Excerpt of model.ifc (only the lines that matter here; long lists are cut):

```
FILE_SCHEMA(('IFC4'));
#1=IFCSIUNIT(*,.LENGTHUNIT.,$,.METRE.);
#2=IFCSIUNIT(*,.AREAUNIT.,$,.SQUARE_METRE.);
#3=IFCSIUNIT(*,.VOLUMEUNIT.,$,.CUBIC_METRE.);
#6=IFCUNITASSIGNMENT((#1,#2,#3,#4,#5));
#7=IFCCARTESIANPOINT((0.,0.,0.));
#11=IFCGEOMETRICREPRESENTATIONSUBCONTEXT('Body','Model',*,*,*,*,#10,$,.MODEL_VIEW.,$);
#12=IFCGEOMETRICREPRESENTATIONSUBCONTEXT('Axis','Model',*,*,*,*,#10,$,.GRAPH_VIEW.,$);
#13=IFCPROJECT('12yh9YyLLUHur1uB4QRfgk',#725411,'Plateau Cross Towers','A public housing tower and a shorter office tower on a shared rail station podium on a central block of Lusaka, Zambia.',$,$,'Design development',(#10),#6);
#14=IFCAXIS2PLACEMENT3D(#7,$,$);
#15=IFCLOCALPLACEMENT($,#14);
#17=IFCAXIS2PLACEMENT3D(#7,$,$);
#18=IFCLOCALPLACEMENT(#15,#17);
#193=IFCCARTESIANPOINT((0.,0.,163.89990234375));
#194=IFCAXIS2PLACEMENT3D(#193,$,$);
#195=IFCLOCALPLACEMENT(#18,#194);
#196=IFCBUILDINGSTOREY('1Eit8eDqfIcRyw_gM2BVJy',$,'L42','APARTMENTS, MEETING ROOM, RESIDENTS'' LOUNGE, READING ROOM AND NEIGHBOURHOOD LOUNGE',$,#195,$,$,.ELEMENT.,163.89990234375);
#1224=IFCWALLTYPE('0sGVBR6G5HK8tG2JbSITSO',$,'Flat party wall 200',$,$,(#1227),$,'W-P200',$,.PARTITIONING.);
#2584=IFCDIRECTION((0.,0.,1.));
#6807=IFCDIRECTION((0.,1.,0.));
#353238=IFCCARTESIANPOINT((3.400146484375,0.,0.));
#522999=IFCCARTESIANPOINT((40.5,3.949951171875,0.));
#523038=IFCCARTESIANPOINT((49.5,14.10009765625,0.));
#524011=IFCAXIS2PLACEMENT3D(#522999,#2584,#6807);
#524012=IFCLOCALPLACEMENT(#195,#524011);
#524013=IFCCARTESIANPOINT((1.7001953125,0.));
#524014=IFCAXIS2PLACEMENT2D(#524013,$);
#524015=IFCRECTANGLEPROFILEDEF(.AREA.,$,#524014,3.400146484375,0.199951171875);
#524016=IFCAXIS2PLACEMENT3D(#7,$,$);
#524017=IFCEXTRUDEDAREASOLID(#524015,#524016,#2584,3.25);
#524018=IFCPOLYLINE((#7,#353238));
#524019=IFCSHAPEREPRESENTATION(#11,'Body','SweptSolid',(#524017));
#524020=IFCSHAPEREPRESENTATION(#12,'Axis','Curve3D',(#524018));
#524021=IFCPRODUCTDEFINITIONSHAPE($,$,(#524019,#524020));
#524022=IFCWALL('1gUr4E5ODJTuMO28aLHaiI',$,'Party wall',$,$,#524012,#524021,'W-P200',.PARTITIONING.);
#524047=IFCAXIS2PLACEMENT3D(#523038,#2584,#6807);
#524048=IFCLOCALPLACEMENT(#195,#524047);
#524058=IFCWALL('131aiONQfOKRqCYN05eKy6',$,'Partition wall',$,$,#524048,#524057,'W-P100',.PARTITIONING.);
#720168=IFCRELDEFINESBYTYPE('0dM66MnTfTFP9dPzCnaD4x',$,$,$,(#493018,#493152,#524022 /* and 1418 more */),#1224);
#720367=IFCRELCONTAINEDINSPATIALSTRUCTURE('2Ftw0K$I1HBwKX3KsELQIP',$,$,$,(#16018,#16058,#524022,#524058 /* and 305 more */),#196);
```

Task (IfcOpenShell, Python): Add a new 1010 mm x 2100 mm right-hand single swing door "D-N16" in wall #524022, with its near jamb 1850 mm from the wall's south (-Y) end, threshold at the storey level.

```python
import numpy as np
import ifcopenshell
import ifcopenshell.api.feature
import ifcopenshell.api.geometry
import ifcopenshell.api.root
import ifcopenshell.api.spatial
import ifcopenshell.geom
import ifcopenshell.util.element
import ifcopenshell.util.placement
import ifcopenshell.util.representation
import ifcopenshell.util.shape
import ifcopenshell.util.unit

model = ifcopenshell.open("model.ifc")
unit_scale = ifcopenshell.util.unit.calculate_unit_scale(model)
settings = ifcopenshell.geom.settings()


def volume(element):
    """Net volume in cubic metres, openings subtracted."""
    shape = ifcopenshell.geom.create_shape(settings, element)
    return ifcopenshell.util.shape.get_volume(shape.geometry)


wall = model.by_id(524022)
storey = ifcopenshell.util.element.get_container(wall, ifc_class="IfcBuildingStorey")
context = ifcopenshell.util.representation.get_context(model, "Model", "Body", "MODEL_VIEW")
before = volume(wall)

width, height, from_end, sill = 1.01, 2.1, 1.85, 0.0  # metres

# The wall runs along its own X axis, and the end named is its -X end.
wall_shape = ifcopenshell.geom.create_shape(settings, wall)
x, y, z = ifcopenshell.util.shape.get_vertices(wall_shape.geometry).T
start = x.min() + from_end
face, thickness = float(y.min()), float(y.max() - y.min())
wall_matrix = ifcopenshell.util.placement.get_local_placement(wall.ObjectPlacement)
level = ifcopenshell.util.placement.get_local_placement(storey.ObjectPlacement)[2, 3]


def in_wall(x, y):
    """Placement at x, y metres in the wall's axes, at sill height."""
    matrix = wall_matrix.copy()
    matrix[:, 3] = wall_matrix @ np.array([x / unit_scale, y / unit_scale, 0.0, 1.0])
    matrix[2, 3] = level + sill / unit_scale
    return matrix


# Opening: a box that overshoots both wall faces by 50 mm.
opening = ifcopenshell.api.root.create_entity(model, ifc_class="IfcOpeningElement", predefined_type="OPENING")
box = ifcopenshell.api.geometry.add_wall_representation(
    model, context=context, length=width, height=height, thickness=thickness + 0.1
)
ifcopenshell.api.geometry.assign_representation(model, product=opening, representation=box)
ifcopenshell.api.geometry.edit_object_placement(model, product=opening, matrix=in_wall(start, face - 0.05), is_si=False)
ifcopenshell.api.feature.add_feature(model, feature=opening, element=wall)

door = ifcopenshell.api.root.create_entity(model, ifc_class="IfcDoor", name="D-N16", predefined_type="DOOR")
door.OverallWidth, door.OverallHeight = width / unit_scale, height / unit_scale
door.OperationType = "SINGLE_SWING_RIGHT"
body = ifcopenshell.api.geometry.add_door_representation(
    model,
    context=context,
    overall_width=door.OverallWidth,
    overall_height=door.OverallHeight,
    operation_type="SINGLE_SWING_RIGHT",
    lining_properties={"LiningDepth": thickness / unit_scale, "ThresholdDepth": thickness / unit_scale},
)
ifcopenshell.api.geometry.assign_representation(model, product=door, representation=body)
ifcopenshell.api.spatial.assign_container(model, products=[door], relating_structure=storey)
ifcopenshell.api.feature.add_filling(model, opening=opening, element=door)

# The lining spans the wall, so the door starts at the wall face.
ifcopenshell.api.geometry.edit_object_placement(model, product=door, matrix=in_wall(start, face), is_si=False)

after = volume(wall)

print(f"wall volume {before:.3f} -> {after:.3f} m3")

model.write("model_edited.ifc")
```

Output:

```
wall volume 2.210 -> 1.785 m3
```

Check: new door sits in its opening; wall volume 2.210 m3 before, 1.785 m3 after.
